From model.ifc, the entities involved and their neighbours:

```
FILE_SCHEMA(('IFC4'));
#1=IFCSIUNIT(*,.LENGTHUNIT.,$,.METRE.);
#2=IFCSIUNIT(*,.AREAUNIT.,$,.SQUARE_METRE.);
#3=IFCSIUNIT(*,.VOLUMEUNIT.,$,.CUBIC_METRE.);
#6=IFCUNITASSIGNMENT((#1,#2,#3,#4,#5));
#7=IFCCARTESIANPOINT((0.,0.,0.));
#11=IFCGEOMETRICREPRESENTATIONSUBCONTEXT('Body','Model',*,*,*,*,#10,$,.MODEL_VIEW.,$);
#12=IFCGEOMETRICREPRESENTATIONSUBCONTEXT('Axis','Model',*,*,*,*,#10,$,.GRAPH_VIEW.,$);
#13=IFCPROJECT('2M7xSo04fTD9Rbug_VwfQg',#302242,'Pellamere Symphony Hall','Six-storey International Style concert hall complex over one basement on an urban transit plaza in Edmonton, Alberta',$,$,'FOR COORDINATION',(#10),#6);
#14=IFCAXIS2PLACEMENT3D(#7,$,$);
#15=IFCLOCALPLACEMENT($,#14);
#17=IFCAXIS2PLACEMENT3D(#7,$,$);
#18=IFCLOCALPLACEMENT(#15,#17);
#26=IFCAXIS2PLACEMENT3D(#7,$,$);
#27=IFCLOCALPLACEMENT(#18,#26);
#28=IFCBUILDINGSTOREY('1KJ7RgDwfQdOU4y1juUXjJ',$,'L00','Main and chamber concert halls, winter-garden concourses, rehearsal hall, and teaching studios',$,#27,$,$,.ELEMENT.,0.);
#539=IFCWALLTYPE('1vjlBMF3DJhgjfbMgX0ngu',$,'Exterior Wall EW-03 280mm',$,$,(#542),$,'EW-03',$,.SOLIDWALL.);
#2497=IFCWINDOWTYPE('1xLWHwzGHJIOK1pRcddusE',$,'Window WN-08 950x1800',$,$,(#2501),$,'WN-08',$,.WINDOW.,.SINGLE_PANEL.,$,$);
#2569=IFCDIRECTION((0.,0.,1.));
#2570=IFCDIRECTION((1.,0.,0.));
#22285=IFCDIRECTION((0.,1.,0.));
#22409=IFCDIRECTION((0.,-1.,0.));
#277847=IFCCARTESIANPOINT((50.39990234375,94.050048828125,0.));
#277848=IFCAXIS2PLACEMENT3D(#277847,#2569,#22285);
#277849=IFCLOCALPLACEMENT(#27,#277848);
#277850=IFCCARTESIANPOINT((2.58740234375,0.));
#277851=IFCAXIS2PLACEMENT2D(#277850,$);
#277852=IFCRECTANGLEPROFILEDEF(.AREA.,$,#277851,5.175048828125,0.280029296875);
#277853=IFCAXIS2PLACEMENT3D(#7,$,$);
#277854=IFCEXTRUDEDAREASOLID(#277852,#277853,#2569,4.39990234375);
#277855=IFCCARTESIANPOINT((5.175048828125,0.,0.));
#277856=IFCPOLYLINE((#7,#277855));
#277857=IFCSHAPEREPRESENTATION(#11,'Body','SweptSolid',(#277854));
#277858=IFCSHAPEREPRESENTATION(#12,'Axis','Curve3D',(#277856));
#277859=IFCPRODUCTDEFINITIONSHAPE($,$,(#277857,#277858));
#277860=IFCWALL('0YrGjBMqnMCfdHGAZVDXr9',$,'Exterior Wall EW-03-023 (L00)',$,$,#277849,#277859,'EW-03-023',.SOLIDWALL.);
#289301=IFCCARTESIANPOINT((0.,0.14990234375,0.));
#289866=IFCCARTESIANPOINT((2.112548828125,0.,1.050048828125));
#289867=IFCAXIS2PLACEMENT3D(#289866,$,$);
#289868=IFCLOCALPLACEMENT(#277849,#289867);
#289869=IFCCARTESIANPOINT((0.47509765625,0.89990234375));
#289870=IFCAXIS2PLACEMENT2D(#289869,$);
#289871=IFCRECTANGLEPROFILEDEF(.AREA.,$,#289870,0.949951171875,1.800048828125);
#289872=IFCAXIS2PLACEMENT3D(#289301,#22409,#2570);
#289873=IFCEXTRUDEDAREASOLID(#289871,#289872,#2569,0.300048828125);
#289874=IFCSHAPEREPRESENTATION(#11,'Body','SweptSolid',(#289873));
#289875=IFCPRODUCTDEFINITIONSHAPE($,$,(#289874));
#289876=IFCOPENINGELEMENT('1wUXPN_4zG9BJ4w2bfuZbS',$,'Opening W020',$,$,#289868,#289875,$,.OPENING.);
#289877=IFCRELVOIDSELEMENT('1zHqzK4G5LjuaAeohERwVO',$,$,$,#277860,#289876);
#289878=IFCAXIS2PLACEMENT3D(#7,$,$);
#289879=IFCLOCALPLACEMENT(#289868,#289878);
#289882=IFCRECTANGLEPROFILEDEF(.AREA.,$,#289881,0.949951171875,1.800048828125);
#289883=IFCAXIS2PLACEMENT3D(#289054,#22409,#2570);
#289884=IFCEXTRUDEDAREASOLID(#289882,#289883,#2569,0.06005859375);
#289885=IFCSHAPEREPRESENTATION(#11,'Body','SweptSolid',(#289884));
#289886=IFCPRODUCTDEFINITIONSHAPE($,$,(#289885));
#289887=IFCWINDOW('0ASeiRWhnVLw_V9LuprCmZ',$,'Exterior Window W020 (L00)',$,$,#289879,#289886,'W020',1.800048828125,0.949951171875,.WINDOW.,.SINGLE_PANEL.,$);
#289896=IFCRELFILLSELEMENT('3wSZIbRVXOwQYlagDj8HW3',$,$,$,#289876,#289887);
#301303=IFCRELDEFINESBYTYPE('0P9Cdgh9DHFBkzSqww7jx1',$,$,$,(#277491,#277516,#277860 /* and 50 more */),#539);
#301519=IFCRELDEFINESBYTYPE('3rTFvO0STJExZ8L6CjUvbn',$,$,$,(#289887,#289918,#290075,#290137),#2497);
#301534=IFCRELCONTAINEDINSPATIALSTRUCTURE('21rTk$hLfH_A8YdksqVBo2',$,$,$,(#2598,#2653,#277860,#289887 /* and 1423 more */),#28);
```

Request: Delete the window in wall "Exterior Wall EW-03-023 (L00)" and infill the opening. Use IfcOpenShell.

```python
import ifcopenshell
import ifcopenshell.api.feature
import ifcopenshell.api.root
import ifcopenshell.geom
import ifcopenshell.util.shape

model = ifcopenshell.open("model.ifc")
settings = ifcopenshell.geom.settings()


def volume(element):
    """Net volume in cubic metres, openings subtracted."""
    shape = ifcopenshell.geom.create_shape(settings, element)
    return ifcopenshell.util.shape.get_volume(shape.geometry)


window = model.by_guid("0ASeiRWhnVLw_V9LuprCmZ")
opening = window.FillsVoids[0].RelatingOpeningElement
wall = opening.VoidsElements[0].RelatingBuildingElement
before = volume(wall)

ifcopenshell.api.root.remove_product(model, product=window)
ifcopenshell.api.feature.remove_feature(model, feature=opening)

after = volume(wall)

print(f"wall volume {before:.3f} -> {after:.3f} m3")

model.write("model_v2.ifc")
```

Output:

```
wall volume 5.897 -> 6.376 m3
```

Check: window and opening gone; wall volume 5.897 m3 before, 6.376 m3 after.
